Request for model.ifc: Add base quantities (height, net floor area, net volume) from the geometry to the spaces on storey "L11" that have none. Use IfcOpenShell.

First a look at what the model holds.

```python
import ifcopenshell
import ifcopenshell.util.element
import ifcopenshell.util.unit

model = ifcopenshell.open("model.ifc")
print(model.schema)
for unit_type in ("LENGTHUNIT", "AREAUNIT", "VOLUMEUNIT"):
    print(unit_type, ifcopenshell.util.unit.calculate_unit_scale(model, unit_type))
storey = next(s for s in model.by_type("IfcBuildingStorey") if s.Name == "L11")
spaces = [e for e in ifcopenshell.util.element.get_decomposition(storey) if e.is_a("IfcSpace")]
for e in sorted(spaces, key=lambda e: e.id()):
    print(e.id(), e.is_a(), e.Name, list(ifcopenshell.util.element.get_psets(e, qtos_only=True)), sep=" | ")
```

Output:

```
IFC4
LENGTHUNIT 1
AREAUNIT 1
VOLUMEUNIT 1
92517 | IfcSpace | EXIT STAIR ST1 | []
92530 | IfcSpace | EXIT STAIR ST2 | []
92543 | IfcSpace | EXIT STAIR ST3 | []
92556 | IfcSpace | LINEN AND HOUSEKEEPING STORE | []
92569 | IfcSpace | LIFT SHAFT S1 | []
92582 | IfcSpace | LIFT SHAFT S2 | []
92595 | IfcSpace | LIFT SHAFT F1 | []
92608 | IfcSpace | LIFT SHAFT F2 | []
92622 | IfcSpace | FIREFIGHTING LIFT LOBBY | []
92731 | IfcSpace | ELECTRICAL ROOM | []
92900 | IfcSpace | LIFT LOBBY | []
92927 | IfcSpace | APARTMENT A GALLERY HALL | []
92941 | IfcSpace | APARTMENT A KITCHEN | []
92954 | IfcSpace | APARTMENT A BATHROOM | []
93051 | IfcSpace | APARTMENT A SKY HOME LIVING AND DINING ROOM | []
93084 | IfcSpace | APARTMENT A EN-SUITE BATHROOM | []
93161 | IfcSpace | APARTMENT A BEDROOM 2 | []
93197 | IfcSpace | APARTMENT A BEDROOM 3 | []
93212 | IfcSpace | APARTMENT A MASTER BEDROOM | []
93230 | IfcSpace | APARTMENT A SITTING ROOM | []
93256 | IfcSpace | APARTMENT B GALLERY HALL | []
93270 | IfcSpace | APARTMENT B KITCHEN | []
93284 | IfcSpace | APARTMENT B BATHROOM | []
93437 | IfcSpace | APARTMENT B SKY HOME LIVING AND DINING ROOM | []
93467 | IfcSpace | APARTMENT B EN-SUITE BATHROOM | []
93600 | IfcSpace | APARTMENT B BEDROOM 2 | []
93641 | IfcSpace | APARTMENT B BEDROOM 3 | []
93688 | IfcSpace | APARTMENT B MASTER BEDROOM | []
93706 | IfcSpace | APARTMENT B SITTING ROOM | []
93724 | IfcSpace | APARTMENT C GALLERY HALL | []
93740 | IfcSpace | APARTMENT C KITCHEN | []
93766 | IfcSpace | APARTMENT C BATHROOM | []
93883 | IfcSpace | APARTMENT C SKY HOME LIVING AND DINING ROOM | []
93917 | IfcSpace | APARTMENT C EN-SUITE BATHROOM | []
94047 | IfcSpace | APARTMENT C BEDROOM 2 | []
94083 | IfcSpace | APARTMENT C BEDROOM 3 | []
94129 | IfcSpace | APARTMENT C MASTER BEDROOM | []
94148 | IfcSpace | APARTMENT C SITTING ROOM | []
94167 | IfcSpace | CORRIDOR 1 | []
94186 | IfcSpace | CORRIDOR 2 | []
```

```python
import ifcopenshell
import ifcopenshell.api.pset
import ifcopenshell.geom
import ifcopenshell.util.element
import ifcopenshell.util.shape
import ifcopenshell.util.unit

model = ifcopenshell.open("model.ifc")
unit_scale = ifcopenshell.util.unit.calculate_unit_scale(model)
area_scale = ifcopenshell.util.unit.calculate_unit_scale(model, "AREAUNIT")
volume_scale = ifcopenshell.util.unit.calculate_unit_scale(model, "VOLUMEUNIT")
settings = ifcopenshell.geom.settings()

storey = next(s for s in model.by_type("IfcBuildingStorey") if s.Name == "L11")
spaces = [e for e in ifcopenshell.util.element.get_decomposition(storey) if e.is_a("IfcSpace")]

for e in sorted(spaces, key=lambda e: e.id()):
    if ifcopenshell.util.element.get_psets(e, qtos_only=True, should_inherit=False):
        continue
    # Geometry comes back in metres, in the element's own axes.
    shape = ifcopenshell.geom.create_shape(settings, e)
    values = {
        "Height": ifcopenshell.util.shape.get_z(shape.geometry) / unit_scale,
        "NetFloorArea": ifcopenshell.util.shape.get_footprint_area(shape.geometry) / area_scale,
        "NetVolume": ifcopenshell.util.shape.get_volume(shape.geometry) / volume_scale,
    }
    qto = ifcopenshell.api.pset.add_qto(model, product=e, name="Qto_SpaceBaseQuantities")
    ifcopenshell.api.pset.edit_qto(model, qto=qto, properties=values)
    print(e.id(), {k: round(v, 3) for k, v in values.items()})

model.write("model-out.ifc")
```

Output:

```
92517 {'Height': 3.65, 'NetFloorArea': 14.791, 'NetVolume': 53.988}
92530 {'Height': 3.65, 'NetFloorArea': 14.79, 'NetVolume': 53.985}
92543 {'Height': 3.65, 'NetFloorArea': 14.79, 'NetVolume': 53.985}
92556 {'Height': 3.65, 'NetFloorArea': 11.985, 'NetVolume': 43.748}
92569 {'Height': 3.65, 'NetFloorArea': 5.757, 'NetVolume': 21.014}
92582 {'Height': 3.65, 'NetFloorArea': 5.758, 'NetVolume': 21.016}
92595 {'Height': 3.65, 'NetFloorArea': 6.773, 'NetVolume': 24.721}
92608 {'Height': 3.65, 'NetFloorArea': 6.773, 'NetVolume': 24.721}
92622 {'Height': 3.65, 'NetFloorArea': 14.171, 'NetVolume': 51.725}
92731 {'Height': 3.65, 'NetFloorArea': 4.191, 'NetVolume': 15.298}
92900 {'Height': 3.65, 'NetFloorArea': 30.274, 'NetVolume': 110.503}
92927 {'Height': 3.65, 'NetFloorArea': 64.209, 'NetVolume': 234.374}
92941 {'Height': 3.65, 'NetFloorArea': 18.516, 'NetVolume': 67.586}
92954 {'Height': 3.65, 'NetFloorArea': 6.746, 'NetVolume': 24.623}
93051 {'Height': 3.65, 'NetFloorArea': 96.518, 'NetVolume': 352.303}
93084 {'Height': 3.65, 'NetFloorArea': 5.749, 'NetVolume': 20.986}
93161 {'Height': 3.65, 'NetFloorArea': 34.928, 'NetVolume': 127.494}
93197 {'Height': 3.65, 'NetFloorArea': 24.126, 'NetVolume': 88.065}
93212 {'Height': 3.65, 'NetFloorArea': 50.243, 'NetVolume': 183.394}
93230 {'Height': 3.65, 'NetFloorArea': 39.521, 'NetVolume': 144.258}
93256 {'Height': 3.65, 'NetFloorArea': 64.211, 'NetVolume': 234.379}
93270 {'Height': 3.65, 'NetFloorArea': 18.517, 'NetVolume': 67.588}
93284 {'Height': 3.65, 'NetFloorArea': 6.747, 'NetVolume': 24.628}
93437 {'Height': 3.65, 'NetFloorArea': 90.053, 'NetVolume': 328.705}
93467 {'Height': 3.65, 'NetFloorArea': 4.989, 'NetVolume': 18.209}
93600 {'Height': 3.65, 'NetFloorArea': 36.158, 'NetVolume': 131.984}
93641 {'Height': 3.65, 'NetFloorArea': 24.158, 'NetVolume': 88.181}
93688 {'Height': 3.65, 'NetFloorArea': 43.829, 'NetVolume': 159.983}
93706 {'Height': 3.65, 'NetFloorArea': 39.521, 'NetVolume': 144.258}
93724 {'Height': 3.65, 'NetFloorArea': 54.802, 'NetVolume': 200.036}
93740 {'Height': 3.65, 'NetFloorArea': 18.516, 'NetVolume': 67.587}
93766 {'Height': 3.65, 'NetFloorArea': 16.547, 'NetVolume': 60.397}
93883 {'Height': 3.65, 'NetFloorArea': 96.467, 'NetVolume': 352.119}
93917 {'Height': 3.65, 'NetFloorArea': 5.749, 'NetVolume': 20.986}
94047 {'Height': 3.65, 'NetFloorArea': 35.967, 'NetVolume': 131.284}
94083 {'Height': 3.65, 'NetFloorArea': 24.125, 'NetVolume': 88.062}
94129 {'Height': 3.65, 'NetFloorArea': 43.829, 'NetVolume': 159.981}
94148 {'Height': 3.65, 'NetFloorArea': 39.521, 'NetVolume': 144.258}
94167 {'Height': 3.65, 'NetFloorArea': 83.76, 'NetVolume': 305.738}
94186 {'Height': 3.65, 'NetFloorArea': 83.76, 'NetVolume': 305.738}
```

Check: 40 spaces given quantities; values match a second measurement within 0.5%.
